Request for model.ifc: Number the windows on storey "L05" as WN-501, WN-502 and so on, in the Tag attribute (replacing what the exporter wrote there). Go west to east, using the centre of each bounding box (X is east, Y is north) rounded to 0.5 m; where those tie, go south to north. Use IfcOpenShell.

First a look at what the model holds.

```python
import ifcopenshell
import ifcopenshell.util.element
import ifcopenshell.util.placement

model = ifcopenshell.open("model.ifc")
print(model.schema)
storey = next(s for s in model.by_type("IfcBuildingStorey") if s.Name == "L05")
windows = [e for e in ifcopenshell.util.element.get_decomposition(storey) if e.is_a("IfcWindow")]
for e in sorted(windows, key=lambda e: e.id()):
    origin = ifcopenshell.util.placement.get_local_placement(e.ObjectPlacement)[:3, 3]
    print(e.id(), e.Tag, e.Name, origin.round(2) + 0.0, sep=" | ")
```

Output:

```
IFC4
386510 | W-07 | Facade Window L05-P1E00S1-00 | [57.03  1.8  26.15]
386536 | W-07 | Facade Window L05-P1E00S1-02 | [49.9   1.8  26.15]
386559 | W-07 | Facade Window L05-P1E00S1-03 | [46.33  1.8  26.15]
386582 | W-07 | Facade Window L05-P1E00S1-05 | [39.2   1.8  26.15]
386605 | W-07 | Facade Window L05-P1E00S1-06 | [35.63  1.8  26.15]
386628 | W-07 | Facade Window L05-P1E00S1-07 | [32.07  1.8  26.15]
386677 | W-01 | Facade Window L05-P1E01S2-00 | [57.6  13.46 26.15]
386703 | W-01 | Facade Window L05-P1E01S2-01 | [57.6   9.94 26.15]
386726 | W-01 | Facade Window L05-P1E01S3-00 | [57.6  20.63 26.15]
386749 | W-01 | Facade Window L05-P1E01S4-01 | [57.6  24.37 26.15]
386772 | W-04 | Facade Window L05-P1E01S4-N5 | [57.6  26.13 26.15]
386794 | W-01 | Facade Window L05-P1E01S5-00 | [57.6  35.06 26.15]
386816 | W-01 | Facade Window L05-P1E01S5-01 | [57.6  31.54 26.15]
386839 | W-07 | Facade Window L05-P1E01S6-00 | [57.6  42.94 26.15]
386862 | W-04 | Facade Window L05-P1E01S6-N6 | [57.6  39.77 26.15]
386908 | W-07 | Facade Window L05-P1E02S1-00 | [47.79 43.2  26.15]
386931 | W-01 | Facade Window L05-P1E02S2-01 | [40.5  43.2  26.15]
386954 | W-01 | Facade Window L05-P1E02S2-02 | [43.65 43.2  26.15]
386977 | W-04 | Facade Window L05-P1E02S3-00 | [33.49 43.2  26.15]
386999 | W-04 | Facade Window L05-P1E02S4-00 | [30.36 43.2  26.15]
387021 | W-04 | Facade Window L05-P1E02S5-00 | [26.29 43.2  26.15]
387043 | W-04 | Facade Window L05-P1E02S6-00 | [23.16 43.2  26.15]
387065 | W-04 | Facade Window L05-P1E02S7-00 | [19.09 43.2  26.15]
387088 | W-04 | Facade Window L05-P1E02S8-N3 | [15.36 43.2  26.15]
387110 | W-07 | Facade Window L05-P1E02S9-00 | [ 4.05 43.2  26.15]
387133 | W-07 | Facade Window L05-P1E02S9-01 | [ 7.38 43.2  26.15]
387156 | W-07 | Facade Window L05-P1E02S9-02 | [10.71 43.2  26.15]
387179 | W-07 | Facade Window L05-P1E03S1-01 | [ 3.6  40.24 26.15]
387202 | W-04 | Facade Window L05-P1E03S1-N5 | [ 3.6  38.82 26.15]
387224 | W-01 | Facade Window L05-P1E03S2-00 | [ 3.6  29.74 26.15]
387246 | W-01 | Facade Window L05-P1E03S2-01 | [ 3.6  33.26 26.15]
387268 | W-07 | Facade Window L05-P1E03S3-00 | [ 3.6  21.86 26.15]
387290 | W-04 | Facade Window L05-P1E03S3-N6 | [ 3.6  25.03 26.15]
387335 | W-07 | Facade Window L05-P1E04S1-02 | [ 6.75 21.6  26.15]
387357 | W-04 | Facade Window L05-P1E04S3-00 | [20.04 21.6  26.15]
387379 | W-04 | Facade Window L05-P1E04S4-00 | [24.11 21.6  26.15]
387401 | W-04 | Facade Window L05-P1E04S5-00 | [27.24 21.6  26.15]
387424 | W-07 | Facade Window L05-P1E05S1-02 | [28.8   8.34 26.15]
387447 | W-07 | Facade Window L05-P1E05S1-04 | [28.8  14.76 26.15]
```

```python
import ifcopenshell
import ifcopenshell.geom
import ifcopenshell.util.element
import ifcopenshell.util.shape

model = ifcopenshell.open("model.ifc")
settings = ifcopenshell.geom.settings()
settings.set("use-world-coords", True)


def centre(element):
    shape = ifcopenshell.geom.create_shape(settings, element)
    return ifcopenshell.util.shape.get_bbox_centroid(shape.geometry)


storey = next(s for s in model.by_type("IfcBuildingStorey") if s.Name == "L05")
windows = [e for e in ifcopenshell.util.element.get_decomposition(storey) if e.is_a("IfcWindow")]

# Insertion points can sit at a corner or the storey origin, so sort by the geometry (in metres).
centres = {e: centre(e) for e in windows}
windows.sort(key=lambda e: (round(centres[e][0] / 0.5), centres[e][1]))

for i, e in enumerate(windows, start=1):
    number = f"WN-5{i:02d}"
    e.Tag = number
    print(e.id(), number)

model.write("model_rev.ifc")
```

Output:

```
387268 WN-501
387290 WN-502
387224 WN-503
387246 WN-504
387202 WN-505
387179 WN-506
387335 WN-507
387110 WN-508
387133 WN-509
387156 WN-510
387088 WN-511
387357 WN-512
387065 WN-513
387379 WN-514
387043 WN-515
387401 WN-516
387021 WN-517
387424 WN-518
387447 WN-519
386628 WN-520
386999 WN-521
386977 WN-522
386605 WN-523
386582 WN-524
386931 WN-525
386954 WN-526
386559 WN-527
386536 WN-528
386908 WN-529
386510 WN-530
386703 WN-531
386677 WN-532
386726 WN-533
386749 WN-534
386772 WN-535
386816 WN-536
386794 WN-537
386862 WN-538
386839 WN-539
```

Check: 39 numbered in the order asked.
